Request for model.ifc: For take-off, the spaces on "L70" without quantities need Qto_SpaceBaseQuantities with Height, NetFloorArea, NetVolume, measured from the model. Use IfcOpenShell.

First a look at what the model holds.

```python
import ifcopenshell
import ifcopenshell.util.element
import ifcopenshell.util.unit

model = ifcopenshell.open("model.ifc")
print(model.schema)
for unit_type in ("LENGTHUNIT", "AREAUNIT", "VOLUMEUNIT"):
    print(unit_type, ifcopenshell.util.unit.calculate_unit_scale(model, unit_type))
storey = next(s for s in model.by_type("IfcBuildingStorey") if s.Name == "L70")
spaces = [e for e in ifcopenshell.util.element.get_decomposition(storey) if e.is_a("IfcSpace")]
for e in sorted(spaces, key=lambda e: e.id()):
    print(e.id(), e.is_a(), e.Name, list(ifcopenshell.util.element.get_psets(e, qtos_only=True)), sep=" | ")
```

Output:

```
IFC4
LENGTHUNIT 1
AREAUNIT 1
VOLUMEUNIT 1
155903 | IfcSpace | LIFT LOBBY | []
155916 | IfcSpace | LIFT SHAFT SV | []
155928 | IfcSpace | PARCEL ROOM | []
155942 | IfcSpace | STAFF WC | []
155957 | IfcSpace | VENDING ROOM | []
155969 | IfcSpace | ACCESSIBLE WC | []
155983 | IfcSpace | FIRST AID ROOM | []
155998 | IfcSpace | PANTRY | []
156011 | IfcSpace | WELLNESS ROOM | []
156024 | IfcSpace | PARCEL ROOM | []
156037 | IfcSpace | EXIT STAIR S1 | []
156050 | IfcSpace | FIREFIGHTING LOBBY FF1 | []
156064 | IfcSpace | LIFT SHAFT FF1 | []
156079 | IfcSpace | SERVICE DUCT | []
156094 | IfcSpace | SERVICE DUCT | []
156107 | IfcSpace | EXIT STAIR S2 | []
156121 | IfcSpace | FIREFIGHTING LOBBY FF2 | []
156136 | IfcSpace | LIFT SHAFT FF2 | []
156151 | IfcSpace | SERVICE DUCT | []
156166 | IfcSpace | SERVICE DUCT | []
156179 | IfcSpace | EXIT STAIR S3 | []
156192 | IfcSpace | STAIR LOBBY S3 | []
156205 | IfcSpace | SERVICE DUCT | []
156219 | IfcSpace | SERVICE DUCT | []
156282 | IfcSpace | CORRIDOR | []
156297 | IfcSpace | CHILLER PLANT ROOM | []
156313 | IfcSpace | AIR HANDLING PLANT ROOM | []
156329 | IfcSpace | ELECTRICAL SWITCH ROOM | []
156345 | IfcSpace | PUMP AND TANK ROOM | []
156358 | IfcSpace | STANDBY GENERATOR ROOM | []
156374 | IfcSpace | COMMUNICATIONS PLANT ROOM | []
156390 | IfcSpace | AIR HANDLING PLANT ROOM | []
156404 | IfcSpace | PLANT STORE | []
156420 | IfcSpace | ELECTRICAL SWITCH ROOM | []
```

```python
import ifcopenshell
import ifcopenshell.api.pset
import ifcopenshell.geom
import ifcopenshell.util.element
import ifcopenshell.util.shape
import ifcopenshell.util.unit

model = ifcopenshell.open("model.ifc")
unit_scale = ifcopenshell.util.unit.calculate_unit_scale(model)
area_scale = ifcopenshell.util.unit.calculate_unit_scale(model, "AREAUNIT")
volume_scale = ifcopenshell.util.unit.calculate_unit_scale(model, "VOLUMEUNIT")
settings = ifcopenshell.geom.settings()

storey = next(s for s in model.by_type("IfcBuildingStorey") if s.Name == "L70")
spaces = [e for e in ifcopenshell.util.element.get_decomposition(storey) if e.is_a("IfcSpace")]

for e in sorted(spaces, key=lambda e: e.id()):
    if ifcopenshell.util.element.get_psets(e, qtos_only=True, should_inherit=False):
        continue
    # Geometry comes back in metres, in the element's own axes.
    shape = ifcopenshell.geom.create_shape(settings, e)
    values = {
        "Height": ifcopenshell.util.shape.get_z(shape.geometry) / unit_scale,
        "NetFloorArea": ifcopenshell.util.shape.get_footprint_area(shape.geometry) / area_scale,
        "NetVolume": ifcopenshell.util.shape.get_volume(shape.geometry) / volume_scale,
    }
    qto = ifcopenshell.api.pset.add_qto(model, product=e, name="Qto_SpaceBaseQuantities")
    ifcopenshell.api.pset.edit_qto(model, qto=qto, properties=values)
    print(e.id(), {k: round(v, 3) for k, v in values.items()})

model.write("model_edited.ifc")
```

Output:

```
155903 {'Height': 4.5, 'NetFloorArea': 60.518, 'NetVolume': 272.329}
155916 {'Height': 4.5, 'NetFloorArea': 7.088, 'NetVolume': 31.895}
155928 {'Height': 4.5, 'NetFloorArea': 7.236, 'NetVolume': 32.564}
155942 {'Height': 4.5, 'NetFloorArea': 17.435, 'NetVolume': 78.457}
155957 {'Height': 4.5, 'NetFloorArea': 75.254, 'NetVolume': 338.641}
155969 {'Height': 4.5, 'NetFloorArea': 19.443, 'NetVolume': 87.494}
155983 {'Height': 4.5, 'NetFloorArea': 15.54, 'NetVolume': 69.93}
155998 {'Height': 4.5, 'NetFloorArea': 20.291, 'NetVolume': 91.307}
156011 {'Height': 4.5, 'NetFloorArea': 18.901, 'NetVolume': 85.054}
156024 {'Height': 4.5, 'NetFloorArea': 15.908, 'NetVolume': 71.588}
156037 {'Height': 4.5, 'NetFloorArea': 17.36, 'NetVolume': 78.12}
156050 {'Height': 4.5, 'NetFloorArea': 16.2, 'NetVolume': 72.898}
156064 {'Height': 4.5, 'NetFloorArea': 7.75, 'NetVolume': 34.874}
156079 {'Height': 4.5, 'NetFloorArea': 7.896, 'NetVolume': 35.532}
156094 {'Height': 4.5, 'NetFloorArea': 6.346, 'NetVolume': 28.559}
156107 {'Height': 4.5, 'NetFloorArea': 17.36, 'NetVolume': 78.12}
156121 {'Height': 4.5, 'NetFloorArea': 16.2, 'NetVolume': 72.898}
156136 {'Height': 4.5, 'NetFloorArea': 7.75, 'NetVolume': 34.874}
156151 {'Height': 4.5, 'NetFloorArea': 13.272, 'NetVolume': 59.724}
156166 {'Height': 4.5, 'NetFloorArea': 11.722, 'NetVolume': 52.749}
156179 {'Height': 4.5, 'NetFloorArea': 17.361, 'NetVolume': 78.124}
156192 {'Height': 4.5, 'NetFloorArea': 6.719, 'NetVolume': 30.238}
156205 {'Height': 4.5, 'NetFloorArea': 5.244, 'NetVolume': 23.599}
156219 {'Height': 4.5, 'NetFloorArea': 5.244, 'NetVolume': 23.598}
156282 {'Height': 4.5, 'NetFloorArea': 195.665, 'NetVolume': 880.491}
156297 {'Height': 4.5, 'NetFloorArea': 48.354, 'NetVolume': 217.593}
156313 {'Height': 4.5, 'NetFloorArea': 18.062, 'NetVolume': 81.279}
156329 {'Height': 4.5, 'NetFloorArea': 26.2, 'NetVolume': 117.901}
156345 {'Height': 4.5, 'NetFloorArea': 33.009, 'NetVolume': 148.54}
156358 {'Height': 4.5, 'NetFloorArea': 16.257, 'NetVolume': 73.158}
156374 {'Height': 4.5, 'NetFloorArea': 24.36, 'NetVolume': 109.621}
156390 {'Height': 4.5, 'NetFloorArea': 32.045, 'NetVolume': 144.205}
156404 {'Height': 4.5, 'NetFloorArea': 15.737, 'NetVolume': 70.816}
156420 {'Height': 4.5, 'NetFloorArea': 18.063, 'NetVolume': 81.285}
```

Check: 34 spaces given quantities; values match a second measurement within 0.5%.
